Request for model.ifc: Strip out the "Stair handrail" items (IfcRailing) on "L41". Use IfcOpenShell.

First a look at what the model holds.

```python
import ifcopenshell
import ifcopenshell.util.element

model = ifcopenshell.open("model.ifc")
print(model.schema)
storey = next(s for s in model.by_type("IfcBuildingStorey") if s.Name == "L41")
railings = [e for e in ifcopenshell.util.element.get_decomposition(storey) if e.is_a("IfcRailing")]
seen = {}
for e in railings:
    element_type = ifcopenshell.util.element.get_type(e)
    name = element_type.Name if element_type not in (None, e) else None
    seen[name] = seen.get(name, 0) + 1
for name, count in sorted(seen.items(), key=str):
    print(count, "x", name)
```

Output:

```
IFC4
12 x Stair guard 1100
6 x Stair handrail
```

```python
import ifcopenshell
import ifcopenshell.api.root
import ifcopenshell.util.element

model = ifcopenshell.open("model.ifc")

storey = next(s for s in model.by_type("IfcBuildingStorey") if s.Name == "L41")
railings = [e for e in ifcopenshell.util.element.get_decomposition(storey) if e.is_a("IfcRailing")]
targets = [e for e in railings if (t := ifcopenshell.util.element.get_type(e)) not in (None, e) and t.Name == "Stair handrail"]

for e in targets:
    ifcopenshell.api.root.remove_product(model, product=e)
print(len(targets), "removed")

model.write("model_edited.ifc")
```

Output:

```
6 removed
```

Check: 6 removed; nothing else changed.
